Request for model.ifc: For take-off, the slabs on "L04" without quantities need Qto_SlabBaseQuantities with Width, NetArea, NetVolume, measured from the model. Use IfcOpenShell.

First a look at what the model holds.

```python
import ifcopenshell
import ifcopenshell.util.element
import ifcopenshell.util.unit

model = ifcopenshell.open("model.ifc")
print(model.schema)
for unit_type in ("LENGTHUNIT", "AREAUNIT", "VOLUMEUNIT"):
    print(unit_type, ifcopenshell.util.unit.calculate_unit_scale(model, unit_type))
storey = next(s for s in model.by_type("IfcBuildingStorey") if s.Name == "L04")
slabs = [e for e in ifcopenshell.util.element.get_decomposition(storey) if e.is_a("IfcSlab")]
for e in sorted(slabs, key=lambda e: e.id()):
    print(e.id(), e.is_a(), e.Name, list(ifcopenshell.util.element.get_psets(e, qtos_only=True)), sep=" | ")
```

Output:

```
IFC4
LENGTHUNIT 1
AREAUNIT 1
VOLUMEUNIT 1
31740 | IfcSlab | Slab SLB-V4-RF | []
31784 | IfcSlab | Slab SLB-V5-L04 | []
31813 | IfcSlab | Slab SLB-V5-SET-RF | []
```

```python
import ifcopenshell
import ifcopenshell.api.pset
import ifcopenshell.geom
import ifcopenshell.util.element
import ifcopenshell.util.shape
import ifcopenshell.util.unit

model = ifcopenshell.open("model.ifc")
unit_scale = ifcopenshell.util.unit.calculate_unit_scale(model)
area_scale = ifcopenshell.util.unit.calculate_unit_scale(model, "AREAUNIT")
volume_scale = ifcopenshell.util.unit.calculate_unit_scale(model, "VOLUMEUNIT")
settings = ifcopenshell.geom.settings()

storey = next(s for s in model.by_type("IfcBuildingStorey") if s.Name == "L04")
slabs = [e for e in ifcopenshell.util.element.get_decomposition(storey) if e.is_a("IfcSlab")]

for e in sorted(slabs, key=lambda e: e.id()):
    if ifcopenshell.util.element.get_psets(e, qtos_only=True, should_inherit=False):
        continue
    # Geometry comes back in metres, in the element's own axes.
    shape = ifcopenshell.geom.create_shape(settings, e)
    values = {
        "Width": ifcopenshell.util.shape.get_z(shape.geometry) / unit_scale,
        "NetArea": ifcopenshell.util.shape.get_footprint_area(shape.geometry) / area_scale,
        "NetVolume": ifcopenshell.util.shape.get_volume(shape.geometry) / volume_scale,
    }
    qto = ifcopenshell.api.pset.add_qto(model, product=e, name="Qto_SlabBaseQuantities")
    ifcopenshell.api.pset.edit_qto(model, qto=qto, properties=values)
    print(e.id(), {k: round(v, 3) for k, v in values.items()})

model.write("model_v2.ifc")
```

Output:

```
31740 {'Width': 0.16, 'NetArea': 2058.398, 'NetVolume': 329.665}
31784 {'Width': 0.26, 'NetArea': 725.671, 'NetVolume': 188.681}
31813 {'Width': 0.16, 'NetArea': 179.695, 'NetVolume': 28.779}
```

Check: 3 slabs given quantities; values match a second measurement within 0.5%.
